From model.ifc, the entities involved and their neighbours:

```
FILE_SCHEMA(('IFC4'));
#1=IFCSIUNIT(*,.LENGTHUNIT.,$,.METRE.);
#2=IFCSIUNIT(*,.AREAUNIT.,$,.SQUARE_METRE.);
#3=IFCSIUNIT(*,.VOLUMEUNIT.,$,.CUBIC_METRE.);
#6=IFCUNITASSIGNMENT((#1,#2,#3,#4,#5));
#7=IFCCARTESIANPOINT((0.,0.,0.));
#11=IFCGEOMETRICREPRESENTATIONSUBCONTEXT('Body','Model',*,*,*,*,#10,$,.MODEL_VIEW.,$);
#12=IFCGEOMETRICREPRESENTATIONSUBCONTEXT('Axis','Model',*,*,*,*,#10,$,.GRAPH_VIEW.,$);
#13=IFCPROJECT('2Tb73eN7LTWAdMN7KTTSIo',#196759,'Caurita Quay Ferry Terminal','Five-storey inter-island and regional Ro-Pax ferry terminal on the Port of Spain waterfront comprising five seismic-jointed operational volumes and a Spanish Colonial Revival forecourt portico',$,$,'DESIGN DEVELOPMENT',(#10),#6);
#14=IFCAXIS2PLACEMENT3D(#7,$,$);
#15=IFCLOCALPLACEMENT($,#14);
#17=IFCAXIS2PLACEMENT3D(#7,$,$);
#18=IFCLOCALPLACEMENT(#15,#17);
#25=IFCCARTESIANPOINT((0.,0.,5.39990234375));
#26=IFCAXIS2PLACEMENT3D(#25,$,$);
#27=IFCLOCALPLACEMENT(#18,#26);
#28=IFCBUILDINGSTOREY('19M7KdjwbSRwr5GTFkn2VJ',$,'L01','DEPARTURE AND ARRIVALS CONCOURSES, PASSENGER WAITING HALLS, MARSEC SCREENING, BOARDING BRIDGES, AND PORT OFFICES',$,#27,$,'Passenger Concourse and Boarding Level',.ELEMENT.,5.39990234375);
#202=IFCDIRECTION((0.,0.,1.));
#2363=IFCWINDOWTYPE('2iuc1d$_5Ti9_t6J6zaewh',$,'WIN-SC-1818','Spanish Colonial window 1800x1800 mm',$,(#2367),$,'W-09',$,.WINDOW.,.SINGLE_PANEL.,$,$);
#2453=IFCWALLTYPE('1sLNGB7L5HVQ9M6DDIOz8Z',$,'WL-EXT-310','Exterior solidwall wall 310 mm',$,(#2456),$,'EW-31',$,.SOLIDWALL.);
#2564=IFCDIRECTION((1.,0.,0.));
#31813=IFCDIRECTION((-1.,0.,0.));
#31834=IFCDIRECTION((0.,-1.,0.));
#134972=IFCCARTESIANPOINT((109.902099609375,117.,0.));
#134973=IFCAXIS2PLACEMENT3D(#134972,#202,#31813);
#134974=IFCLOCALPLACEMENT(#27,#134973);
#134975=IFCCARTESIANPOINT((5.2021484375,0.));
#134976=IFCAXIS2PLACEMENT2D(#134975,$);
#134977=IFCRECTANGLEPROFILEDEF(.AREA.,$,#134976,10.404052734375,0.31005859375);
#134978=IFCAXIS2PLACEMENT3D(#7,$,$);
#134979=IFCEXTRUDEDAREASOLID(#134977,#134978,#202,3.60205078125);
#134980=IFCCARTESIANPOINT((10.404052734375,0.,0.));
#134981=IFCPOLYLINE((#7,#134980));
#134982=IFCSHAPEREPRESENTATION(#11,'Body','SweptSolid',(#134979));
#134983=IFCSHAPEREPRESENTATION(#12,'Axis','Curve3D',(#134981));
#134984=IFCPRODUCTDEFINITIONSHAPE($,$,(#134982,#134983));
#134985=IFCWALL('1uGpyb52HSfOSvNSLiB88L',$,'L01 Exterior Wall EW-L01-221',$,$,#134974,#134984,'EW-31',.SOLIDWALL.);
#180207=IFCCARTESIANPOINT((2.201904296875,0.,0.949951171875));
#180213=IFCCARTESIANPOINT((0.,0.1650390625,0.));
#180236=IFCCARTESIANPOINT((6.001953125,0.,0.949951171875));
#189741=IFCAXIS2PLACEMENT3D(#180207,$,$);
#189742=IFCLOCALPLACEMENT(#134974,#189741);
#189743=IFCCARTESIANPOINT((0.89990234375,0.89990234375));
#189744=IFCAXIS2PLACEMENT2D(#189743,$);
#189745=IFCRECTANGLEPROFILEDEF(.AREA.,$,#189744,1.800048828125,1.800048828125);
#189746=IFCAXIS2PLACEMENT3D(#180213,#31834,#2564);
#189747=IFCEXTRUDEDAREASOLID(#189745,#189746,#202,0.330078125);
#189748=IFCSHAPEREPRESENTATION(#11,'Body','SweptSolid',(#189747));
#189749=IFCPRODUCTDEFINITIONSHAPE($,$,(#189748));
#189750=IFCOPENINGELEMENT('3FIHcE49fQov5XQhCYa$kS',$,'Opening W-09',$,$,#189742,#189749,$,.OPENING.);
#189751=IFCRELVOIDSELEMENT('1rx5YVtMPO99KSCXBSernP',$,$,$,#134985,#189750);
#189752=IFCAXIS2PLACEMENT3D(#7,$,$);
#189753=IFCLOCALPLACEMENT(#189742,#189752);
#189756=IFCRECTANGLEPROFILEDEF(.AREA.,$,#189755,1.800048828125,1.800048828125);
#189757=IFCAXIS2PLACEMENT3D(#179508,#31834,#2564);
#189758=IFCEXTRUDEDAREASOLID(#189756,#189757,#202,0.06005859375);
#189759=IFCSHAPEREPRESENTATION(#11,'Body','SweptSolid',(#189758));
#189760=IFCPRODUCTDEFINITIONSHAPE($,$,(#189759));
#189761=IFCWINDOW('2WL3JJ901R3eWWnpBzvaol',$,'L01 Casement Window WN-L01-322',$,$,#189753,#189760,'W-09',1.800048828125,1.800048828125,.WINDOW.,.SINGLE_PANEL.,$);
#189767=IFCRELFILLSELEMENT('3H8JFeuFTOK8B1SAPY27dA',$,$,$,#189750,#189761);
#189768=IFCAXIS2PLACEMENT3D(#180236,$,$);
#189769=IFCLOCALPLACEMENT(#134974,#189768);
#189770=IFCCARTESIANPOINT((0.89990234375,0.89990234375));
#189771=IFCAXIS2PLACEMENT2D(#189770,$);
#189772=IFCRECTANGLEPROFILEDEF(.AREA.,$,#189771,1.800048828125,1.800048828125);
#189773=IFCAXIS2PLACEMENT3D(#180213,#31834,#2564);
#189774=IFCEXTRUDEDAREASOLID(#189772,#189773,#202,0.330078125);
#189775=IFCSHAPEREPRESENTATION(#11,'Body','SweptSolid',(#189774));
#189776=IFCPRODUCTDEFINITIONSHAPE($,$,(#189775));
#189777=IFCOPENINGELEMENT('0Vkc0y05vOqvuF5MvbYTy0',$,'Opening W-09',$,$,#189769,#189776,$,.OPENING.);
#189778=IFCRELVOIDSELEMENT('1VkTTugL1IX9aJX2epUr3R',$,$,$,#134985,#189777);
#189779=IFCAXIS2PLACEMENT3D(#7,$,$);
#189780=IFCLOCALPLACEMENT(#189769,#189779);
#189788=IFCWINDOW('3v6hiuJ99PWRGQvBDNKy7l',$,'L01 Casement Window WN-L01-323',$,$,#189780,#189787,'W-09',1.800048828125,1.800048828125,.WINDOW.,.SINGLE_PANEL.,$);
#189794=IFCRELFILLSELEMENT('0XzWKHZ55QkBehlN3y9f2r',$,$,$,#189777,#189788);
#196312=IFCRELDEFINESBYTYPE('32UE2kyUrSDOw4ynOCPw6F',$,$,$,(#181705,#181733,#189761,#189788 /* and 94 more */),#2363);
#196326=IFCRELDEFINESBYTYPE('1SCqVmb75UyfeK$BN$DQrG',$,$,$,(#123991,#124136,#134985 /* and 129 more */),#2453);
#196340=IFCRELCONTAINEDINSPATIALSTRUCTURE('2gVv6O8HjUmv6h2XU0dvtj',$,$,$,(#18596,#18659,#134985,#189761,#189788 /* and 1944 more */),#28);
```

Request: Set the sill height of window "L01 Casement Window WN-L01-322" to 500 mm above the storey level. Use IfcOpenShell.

```python
import numpy as np
import ifcopenshell
import ifcopenshell.api.geometry
import ifcopenshell.geom
import ifcopenshell.util.element
import ifcopenshell.util.placement
import ifcopenshell.util.shape
import ifcopenshell.util.unit

model = ifcopenshell.open("model.ifc")
unit_scale = ifcopenshell.util.unit.calculate_unit_scale(model)

window = model.by_id(189761)
opening = window.FillsVoids[0].RelatingOpeningElement
storey = ifcopenshell.util.element.get_container(window, ifc_class="IfcBuildingStorey")
level = ifcopenshell.util.placement.get_local_placement(storey.ObjectPlacement)[2, 3]

# The opening's origin need not be at the sill, so measure its lowest point.
shape = ifcopenshell.geom.create_shape(ifcopenshell.geom.settings(), opening)
bottom = ifcopenshell.util.shape.get_shape_bottom_elevation(shape, shape.geometry) / unit_scale
dz = level + 0.5 / unit_scale - bottom

shift = np.array([0.0, 0.0, dz])
# The window is placed relative to its opening, so it follows when the opening moves.
matrix = ifcopenshell.util.placement.get_local_placement(opening.ObjectPlacement)
matrix[:3, 3] += shift
ifcopenshell.api.geometry.edit_object_placement(
    model, product=opening, matrix=matrix, is_si=False, should_transform_children=True
)

print(f"moved by {dz * unit_scale:+.3f} m")

model.write("model-out.ifc")
```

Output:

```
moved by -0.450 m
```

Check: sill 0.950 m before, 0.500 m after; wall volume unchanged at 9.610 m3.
